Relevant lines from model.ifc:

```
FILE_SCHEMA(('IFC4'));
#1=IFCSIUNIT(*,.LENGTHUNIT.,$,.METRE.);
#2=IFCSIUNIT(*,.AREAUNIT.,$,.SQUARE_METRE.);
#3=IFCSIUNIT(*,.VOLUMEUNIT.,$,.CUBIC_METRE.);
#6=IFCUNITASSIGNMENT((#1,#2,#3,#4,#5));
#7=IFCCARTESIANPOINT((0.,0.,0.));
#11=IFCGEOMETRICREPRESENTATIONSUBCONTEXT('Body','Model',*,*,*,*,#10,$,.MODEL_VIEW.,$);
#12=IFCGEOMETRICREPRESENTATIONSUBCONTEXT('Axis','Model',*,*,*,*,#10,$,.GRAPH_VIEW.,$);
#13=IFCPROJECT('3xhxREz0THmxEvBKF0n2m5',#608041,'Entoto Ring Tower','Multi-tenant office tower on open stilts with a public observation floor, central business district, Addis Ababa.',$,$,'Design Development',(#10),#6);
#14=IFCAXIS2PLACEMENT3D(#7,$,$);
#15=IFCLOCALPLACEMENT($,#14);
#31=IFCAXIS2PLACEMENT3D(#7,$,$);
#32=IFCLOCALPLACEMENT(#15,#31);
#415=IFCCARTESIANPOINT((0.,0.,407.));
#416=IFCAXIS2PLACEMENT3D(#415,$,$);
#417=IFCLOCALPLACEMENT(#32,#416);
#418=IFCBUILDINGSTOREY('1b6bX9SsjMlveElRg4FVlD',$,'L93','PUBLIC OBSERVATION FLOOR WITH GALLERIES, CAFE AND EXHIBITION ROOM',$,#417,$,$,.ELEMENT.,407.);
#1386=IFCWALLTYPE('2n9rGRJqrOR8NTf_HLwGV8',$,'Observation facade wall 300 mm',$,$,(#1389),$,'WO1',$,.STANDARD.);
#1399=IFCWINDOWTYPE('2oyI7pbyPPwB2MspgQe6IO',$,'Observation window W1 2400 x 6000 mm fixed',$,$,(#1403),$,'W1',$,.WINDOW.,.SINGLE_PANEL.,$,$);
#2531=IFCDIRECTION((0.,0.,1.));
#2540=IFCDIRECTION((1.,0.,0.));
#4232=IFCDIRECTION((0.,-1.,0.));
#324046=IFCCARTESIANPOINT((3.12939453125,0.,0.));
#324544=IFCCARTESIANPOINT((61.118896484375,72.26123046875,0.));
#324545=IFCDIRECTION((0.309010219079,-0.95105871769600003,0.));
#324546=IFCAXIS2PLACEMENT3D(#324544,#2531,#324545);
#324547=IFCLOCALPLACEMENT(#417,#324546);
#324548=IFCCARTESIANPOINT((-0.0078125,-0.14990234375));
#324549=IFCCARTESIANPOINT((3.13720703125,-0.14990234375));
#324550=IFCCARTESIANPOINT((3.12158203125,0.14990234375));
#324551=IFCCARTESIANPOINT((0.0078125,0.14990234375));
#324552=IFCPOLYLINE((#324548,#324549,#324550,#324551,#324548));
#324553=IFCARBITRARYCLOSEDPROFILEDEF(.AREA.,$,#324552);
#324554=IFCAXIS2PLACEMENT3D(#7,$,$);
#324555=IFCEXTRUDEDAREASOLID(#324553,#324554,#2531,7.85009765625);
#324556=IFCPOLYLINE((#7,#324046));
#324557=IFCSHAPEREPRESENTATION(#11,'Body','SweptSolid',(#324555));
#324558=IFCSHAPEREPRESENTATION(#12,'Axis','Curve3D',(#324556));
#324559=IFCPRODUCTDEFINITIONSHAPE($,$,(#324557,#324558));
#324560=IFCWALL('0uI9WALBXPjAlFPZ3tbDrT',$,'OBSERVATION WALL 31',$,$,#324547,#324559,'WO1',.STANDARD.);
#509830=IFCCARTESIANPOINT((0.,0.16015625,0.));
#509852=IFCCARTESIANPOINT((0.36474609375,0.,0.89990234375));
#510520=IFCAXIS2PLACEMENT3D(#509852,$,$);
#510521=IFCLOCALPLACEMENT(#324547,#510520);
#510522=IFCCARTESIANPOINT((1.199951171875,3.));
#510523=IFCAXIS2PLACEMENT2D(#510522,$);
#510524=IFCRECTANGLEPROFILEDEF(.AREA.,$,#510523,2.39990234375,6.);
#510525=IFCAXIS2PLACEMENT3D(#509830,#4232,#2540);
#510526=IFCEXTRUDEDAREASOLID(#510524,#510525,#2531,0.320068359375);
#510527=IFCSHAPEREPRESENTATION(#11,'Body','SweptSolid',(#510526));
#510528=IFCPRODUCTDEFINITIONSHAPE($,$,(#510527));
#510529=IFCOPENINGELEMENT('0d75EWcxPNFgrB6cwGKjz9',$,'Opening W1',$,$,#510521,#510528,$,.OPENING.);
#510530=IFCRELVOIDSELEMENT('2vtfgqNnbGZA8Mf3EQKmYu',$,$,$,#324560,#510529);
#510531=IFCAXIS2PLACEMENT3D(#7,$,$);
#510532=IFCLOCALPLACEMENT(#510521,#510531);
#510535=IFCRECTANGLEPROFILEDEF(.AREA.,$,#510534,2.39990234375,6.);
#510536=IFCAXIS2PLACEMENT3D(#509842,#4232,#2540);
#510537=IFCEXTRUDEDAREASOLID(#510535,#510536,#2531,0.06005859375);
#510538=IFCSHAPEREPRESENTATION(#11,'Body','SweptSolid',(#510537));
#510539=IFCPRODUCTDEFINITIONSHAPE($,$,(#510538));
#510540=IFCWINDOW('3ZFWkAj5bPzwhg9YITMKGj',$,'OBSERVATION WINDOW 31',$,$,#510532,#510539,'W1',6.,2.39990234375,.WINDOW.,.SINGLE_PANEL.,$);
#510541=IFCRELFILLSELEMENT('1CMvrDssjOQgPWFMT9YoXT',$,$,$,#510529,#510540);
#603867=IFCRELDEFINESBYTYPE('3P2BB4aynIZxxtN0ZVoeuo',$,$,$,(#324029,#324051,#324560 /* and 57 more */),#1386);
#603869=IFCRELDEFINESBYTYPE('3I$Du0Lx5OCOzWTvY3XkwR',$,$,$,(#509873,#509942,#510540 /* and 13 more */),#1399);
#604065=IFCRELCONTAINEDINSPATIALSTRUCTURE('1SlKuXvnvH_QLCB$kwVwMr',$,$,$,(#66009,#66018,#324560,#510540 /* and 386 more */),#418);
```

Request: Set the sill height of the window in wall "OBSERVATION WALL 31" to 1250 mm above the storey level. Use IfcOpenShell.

```python
import numpy as np
import ifcopenshell
import ifcopenshell.api.geometry
import ifcopenshell.geom
import ifcopenshell.util.element
import ifcopenshell.util.placement
import ifcopenshell.util.shape
import ifcopenshell.util.unit

model = ifcopenshell.open("model.ifc")
unit_scale = ifcopenshell.util.unit.calculate_unit_scale(model)

window = model.by_id(510540)
opening = window.FillsVoids[0].RelatingOpeningElement
storey = ifcopenshell.util.element.get_container(window, ifc_class="IfcBuildingStorey")
level = ifcopenshell.util.placement.get_local_placement(storey.ObjectPlacement)[2, 3]

# The opening's origin need not be at the sill, so measure its lowest point.
shape = ifcopenshell.geom.create_shape(ifcopenshell.geom.settings(), opening)
bottom = ifcopenshell.util.shape.get_shape_bottom_elevation(shape, shape.geometry) / unit_scale
dz = level + 1.25 / unit_scale - bottom

shift = np.array([0.0, 0.0, dz])
# The window is placed relative to its opening, so it follows when the opening moves.
matrix = ifcopenshell.util.placement.get_local_placement(opening.ObjectPlacement)
matrix[:3, 3] += shift
ifcopenshell.api.geometry.edit_object_placement(
    model, product=opening, matrix=matrix, is_si=False, should_transform_children=True
)

print(f"moved by {dz * unit_scale:+.3f} m")

model.write("model_updated.ifc")
```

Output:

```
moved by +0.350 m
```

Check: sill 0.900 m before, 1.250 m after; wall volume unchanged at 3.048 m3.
